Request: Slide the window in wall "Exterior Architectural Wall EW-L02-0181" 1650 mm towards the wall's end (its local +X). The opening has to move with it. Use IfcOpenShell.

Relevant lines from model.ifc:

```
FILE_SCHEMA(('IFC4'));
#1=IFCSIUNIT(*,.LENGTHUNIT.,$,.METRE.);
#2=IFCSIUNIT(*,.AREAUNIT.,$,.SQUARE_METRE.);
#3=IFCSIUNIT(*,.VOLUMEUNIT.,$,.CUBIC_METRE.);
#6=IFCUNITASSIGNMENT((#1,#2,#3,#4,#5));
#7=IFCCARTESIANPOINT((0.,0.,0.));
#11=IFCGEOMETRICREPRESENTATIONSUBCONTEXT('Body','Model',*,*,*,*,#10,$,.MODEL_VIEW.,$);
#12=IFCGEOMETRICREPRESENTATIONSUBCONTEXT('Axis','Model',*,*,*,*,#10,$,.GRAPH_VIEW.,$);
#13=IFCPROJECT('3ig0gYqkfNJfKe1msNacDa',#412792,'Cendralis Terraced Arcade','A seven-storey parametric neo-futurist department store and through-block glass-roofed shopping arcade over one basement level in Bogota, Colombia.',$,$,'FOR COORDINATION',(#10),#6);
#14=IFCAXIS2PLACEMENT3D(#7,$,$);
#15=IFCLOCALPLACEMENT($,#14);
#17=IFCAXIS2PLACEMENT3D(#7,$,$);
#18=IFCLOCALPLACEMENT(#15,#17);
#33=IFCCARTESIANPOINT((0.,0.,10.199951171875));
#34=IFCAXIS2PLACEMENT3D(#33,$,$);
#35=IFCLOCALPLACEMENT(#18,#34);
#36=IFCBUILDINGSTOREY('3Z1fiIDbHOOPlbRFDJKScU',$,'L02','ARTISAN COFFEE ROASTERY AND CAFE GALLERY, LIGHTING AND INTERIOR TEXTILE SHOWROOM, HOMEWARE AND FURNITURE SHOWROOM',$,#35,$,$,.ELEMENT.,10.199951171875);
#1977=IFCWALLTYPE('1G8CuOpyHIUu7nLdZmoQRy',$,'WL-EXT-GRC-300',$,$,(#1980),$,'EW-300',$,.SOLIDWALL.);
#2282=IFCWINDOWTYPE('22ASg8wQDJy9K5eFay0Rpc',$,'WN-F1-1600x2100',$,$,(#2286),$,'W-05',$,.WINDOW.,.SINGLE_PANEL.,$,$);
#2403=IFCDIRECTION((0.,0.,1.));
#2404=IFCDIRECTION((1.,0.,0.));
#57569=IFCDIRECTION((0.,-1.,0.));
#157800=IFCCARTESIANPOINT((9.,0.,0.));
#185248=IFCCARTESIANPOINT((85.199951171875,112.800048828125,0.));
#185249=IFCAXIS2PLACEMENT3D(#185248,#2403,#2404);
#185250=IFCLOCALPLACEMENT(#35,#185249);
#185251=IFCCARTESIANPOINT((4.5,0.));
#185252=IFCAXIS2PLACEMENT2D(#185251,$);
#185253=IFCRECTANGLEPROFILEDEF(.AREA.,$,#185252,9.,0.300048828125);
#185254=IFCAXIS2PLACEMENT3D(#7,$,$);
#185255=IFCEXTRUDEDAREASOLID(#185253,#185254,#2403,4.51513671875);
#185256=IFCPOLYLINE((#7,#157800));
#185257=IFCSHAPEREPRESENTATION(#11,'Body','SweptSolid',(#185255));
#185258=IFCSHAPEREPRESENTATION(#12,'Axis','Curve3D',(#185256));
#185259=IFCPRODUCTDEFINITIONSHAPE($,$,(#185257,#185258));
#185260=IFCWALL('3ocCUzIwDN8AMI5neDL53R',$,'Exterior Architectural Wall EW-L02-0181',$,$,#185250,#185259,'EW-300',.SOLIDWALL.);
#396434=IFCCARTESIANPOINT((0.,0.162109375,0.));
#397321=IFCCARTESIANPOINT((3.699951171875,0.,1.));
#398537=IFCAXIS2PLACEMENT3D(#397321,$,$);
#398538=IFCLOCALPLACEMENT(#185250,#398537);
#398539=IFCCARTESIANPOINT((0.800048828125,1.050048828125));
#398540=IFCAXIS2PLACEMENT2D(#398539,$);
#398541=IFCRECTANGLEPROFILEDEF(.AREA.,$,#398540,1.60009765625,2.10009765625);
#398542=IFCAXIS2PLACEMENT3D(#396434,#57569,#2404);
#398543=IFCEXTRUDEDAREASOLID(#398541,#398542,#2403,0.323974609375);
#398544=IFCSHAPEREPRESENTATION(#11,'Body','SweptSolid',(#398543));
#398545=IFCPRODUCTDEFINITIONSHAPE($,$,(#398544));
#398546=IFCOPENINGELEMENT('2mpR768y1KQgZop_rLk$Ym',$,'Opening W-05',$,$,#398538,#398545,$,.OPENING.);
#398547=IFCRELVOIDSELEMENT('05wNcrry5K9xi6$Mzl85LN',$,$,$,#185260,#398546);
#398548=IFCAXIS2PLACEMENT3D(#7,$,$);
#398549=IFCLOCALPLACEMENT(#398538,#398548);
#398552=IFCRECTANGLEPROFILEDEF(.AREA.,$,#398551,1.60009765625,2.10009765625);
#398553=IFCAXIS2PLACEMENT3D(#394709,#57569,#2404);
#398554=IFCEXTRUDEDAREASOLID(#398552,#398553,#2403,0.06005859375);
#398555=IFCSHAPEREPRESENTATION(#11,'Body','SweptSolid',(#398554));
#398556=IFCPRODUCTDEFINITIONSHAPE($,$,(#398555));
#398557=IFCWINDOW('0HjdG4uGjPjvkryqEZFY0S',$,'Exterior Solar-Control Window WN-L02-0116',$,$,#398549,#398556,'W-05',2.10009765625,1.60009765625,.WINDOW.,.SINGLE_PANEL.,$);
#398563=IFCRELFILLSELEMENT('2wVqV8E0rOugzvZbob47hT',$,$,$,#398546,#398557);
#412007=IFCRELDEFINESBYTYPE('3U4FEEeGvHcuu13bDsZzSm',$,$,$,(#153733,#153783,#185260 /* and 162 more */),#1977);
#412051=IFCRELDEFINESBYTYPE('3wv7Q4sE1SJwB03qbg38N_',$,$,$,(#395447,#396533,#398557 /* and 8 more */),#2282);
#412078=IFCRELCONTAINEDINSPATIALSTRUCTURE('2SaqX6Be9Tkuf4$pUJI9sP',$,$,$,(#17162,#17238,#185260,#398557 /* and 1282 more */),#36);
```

```python
import ifcopenshell
import ifcopenshell.api.geometry
import ifcopenshell.util.placement

model = ifcopenshell.open("model.ifc")

window = model.by_guid("0HjdG4uGjPjvkryqEZFY0S")
opening = window.FillsVoids[0].RelatingOpeningElement
wall = opening.VoidsElements[0].RelatingBuildingElement

wall_matrix = ifcopenshell.util.placement.get_local_placement(wall.ObjectPlacement)
shift = wall_matrix[:3, 0] * 1.65
before = ifcopenshell.util.placement.get_local_placement(window.ObjectPlacement)[:3, 3].copy()

# The window is placed relative to its opening, so it follows when the opening moves.
matrix = ifcopenshell.util.placement.get_local_placement(opening.ObjectPlacement)
matrix[:3, 3] += shift
ifcopenshell.api.geometry.edit_object_placement(
    model, product=opening, matrix=matrix, is_si=False, should_transform_children=True
)

after = ifcopenshell.util.placement.get_local_placement(window.ObjectPlacement)[:3, 3]
print("window moved by", (after - before).round(3) + 0.0)

model.write("model_edited.ifc")
```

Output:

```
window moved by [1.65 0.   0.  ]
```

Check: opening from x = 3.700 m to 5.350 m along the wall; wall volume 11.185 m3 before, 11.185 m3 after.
